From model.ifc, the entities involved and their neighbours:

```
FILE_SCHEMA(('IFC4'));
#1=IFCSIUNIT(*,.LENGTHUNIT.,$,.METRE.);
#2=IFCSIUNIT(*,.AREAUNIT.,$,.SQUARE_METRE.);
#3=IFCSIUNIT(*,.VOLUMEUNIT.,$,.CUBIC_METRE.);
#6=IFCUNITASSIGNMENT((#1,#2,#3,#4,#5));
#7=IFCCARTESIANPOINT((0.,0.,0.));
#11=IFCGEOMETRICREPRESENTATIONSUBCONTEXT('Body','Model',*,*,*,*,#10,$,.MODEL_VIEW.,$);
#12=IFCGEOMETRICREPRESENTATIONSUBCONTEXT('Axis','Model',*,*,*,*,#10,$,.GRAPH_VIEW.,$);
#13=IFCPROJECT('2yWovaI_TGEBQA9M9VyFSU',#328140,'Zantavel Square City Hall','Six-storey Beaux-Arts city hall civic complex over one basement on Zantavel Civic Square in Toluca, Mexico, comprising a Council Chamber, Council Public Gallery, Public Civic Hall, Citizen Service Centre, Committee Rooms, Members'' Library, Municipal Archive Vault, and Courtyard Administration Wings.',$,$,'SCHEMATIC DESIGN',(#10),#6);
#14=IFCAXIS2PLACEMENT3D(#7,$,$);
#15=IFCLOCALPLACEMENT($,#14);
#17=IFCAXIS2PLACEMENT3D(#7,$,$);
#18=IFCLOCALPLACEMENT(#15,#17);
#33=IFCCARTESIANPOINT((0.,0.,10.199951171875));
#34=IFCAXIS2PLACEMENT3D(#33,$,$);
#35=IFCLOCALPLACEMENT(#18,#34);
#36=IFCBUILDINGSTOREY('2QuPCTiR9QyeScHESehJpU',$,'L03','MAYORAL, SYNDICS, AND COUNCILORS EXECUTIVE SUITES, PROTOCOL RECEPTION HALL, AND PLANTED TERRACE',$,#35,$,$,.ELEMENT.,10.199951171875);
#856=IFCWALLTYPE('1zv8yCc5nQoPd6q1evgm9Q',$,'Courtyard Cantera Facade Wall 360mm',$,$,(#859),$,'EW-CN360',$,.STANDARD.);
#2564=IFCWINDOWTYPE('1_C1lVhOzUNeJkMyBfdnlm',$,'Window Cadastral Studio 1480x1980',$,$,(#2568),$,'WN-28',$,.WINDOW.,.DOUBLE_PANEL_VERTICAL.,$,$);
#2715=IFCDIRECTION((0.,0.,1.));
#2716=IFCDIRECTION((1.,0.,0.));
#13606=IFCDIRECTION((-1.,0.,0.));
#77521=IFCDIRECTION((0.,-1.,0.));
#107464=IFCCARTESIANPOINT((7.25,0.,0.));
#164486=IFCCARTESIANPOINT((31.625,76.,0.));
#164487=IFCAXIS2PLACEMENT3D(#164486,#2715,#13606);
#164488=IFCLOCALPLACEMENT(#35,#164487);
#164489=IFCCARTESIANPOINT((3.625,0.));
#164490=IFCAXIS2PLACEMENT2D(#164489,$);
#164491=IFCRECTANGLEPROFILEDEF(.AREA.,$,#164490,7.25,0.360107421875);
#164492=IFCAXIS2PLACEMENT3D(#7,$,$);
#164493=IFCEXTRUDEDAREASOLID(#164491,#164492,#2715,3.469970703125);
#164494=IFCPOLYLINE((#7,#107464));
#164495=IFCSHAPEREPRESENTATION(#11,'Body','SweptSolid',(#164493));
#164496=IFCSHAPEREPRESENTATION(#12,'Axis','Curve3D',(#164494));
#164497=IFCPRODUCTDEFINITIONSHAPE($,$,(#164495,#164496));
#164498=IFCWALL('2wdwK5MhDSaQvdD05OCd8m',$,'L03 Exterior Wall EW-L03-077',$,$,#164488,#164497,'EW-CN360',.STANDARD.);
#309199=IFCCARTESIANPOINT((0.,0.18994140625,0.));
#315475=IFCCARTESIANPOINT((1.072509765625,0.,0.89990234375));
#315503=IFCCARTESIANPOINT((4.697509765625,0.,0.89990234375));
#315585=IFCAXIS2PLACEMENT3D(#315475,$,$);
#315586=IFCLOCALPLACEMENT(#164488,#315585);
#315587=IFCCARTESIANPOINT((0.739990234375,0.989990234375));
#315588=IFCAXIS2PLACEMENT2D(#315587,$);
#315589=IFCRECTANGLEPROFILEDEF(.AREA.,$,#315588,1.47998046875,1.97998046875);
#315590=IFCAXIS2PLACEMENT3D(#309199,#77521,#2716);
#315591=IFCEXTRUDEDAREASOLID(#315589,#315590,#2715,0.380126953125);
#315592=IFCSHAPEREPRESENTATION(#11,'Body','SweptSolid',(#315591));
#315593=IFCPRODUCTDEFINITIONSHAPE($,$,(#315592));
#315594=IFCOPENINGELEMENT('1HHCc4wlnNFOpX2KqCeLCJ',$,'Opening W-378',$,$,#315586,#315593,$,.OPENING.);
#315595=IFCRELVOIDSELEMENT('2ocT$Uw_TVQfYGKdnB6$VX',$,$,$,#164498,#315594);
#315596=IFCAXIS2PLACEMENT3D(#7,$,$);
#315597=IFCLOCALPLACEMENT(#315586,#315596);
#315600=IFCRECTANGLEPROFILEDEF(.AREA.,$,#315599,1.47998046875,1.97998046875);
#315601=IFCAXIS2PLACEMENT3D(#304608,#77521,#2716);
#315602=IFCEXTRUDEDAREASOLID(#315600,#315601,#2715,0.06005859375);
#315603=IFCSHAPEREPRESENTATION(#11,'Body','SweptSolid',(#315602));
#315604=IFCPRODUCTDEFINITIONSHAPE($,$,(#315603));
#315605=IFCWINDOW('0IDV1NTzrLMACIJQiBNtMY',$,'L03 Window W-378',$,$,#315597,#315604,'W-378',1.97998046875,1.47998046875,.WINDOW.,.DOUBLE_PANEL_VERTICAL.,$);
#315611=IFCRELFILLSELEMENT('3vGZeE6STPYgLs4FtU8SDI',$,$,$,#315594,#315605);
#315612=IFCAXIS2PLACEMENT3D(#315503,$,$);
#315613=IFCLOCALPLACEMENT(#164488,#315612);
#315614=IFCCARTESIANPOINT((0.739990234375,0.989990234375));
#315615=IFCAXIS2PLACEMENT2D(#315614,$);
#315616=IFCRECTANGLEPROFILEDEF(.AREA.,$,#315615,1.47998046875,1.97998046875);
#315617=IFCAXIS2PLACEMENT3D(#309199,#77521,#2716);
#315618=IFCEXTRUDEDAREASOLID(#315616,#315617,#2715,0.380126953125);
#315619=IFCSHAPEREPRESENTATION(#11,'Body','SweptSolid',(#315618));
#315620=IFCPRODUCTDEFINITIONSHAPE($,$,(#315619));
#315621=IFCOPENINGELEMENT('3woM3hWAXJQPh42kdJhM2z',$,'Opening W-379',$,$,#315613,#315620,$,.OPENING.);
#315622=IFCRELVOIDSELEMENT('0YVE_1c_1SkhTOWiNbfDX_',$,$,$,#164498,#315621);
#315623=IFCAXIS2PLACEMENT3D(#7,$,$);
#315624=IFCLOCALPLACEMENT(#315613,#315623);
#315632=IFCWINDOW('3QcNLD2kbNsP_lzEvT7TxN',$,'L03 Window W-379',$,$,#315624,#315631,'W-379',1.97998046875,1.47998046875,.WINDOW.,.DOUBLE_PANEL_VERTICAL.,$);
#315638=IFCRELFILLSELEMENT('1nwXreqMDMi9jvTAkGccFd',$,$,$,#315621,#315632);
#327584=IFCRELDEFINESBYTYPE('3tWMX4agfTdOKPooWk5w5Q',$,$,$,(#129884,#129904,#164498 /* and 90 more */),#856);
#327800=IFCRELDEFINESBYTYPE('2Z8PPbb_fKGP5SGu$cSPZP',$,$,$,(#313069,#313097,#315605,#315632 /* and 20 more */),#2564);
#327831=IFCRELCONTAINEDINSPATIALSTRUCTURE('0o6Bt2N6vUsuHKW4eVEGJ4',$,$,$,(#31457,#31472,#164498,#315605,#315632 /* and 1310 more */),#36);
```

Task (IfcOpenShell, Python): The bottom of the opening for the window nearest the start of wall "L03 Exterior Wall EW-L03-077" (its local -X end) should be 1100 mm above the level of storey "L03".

```python
import numpy as np
import ifcopenshell
import ifcopenshell.api.geometry
import ifcopenshell.geom
import ifcopenshell.util.element
import ifcopenshell.util.placement
import ifcopenshell.util.shape
import ifcopenshell.util.unit

model = ifcopenshell.open("model.ifc")
unit_scale = ifcopenshell.util.unit.calculate_unit_scale(model)

window = model.by_id(315605)
opening = window.FillsVoids[0].RelatingOpeningElement
storey = ifcopenshell.util.element.get_container(window, ifc_class="IfcBuildingStorey")
level = ifcopenshell.util.placement.get_local_placement(storey.ObjectPlacement)[2, 3]

# The opening's origin need not be at the sill, so measure its lowest point.
shape = ifcopenshell.geom.create_shape(ifcopenshell.geom.settings(), opening)
bottom = ifcopenshell.util.shape.get_shape_bottom_elevation(shape, shape.geometry) / unit_scale
dz = level + 1.1 / unit_scale - bottom

shift = np.array([0.0, 0.0, dz])
# The window is placed relative to its opening, so it follows when the opening moves.
matrix = ifcopenshell.util.placement.get_local_placement(opening.ObjectPlacement)
matrix[:3, 3] += shift
ifcopenshell.api.geometry.edit_object_placement(
    model, product=opening, matrix=matrix, is_si=False, should_transform_children=True
)

print(f"moved by {dz * unit_scale:+.3f} m")

model.write("model-out.ifc")
```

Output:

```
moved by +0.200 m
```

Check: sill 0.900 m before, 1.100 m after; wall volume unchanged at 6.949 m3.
